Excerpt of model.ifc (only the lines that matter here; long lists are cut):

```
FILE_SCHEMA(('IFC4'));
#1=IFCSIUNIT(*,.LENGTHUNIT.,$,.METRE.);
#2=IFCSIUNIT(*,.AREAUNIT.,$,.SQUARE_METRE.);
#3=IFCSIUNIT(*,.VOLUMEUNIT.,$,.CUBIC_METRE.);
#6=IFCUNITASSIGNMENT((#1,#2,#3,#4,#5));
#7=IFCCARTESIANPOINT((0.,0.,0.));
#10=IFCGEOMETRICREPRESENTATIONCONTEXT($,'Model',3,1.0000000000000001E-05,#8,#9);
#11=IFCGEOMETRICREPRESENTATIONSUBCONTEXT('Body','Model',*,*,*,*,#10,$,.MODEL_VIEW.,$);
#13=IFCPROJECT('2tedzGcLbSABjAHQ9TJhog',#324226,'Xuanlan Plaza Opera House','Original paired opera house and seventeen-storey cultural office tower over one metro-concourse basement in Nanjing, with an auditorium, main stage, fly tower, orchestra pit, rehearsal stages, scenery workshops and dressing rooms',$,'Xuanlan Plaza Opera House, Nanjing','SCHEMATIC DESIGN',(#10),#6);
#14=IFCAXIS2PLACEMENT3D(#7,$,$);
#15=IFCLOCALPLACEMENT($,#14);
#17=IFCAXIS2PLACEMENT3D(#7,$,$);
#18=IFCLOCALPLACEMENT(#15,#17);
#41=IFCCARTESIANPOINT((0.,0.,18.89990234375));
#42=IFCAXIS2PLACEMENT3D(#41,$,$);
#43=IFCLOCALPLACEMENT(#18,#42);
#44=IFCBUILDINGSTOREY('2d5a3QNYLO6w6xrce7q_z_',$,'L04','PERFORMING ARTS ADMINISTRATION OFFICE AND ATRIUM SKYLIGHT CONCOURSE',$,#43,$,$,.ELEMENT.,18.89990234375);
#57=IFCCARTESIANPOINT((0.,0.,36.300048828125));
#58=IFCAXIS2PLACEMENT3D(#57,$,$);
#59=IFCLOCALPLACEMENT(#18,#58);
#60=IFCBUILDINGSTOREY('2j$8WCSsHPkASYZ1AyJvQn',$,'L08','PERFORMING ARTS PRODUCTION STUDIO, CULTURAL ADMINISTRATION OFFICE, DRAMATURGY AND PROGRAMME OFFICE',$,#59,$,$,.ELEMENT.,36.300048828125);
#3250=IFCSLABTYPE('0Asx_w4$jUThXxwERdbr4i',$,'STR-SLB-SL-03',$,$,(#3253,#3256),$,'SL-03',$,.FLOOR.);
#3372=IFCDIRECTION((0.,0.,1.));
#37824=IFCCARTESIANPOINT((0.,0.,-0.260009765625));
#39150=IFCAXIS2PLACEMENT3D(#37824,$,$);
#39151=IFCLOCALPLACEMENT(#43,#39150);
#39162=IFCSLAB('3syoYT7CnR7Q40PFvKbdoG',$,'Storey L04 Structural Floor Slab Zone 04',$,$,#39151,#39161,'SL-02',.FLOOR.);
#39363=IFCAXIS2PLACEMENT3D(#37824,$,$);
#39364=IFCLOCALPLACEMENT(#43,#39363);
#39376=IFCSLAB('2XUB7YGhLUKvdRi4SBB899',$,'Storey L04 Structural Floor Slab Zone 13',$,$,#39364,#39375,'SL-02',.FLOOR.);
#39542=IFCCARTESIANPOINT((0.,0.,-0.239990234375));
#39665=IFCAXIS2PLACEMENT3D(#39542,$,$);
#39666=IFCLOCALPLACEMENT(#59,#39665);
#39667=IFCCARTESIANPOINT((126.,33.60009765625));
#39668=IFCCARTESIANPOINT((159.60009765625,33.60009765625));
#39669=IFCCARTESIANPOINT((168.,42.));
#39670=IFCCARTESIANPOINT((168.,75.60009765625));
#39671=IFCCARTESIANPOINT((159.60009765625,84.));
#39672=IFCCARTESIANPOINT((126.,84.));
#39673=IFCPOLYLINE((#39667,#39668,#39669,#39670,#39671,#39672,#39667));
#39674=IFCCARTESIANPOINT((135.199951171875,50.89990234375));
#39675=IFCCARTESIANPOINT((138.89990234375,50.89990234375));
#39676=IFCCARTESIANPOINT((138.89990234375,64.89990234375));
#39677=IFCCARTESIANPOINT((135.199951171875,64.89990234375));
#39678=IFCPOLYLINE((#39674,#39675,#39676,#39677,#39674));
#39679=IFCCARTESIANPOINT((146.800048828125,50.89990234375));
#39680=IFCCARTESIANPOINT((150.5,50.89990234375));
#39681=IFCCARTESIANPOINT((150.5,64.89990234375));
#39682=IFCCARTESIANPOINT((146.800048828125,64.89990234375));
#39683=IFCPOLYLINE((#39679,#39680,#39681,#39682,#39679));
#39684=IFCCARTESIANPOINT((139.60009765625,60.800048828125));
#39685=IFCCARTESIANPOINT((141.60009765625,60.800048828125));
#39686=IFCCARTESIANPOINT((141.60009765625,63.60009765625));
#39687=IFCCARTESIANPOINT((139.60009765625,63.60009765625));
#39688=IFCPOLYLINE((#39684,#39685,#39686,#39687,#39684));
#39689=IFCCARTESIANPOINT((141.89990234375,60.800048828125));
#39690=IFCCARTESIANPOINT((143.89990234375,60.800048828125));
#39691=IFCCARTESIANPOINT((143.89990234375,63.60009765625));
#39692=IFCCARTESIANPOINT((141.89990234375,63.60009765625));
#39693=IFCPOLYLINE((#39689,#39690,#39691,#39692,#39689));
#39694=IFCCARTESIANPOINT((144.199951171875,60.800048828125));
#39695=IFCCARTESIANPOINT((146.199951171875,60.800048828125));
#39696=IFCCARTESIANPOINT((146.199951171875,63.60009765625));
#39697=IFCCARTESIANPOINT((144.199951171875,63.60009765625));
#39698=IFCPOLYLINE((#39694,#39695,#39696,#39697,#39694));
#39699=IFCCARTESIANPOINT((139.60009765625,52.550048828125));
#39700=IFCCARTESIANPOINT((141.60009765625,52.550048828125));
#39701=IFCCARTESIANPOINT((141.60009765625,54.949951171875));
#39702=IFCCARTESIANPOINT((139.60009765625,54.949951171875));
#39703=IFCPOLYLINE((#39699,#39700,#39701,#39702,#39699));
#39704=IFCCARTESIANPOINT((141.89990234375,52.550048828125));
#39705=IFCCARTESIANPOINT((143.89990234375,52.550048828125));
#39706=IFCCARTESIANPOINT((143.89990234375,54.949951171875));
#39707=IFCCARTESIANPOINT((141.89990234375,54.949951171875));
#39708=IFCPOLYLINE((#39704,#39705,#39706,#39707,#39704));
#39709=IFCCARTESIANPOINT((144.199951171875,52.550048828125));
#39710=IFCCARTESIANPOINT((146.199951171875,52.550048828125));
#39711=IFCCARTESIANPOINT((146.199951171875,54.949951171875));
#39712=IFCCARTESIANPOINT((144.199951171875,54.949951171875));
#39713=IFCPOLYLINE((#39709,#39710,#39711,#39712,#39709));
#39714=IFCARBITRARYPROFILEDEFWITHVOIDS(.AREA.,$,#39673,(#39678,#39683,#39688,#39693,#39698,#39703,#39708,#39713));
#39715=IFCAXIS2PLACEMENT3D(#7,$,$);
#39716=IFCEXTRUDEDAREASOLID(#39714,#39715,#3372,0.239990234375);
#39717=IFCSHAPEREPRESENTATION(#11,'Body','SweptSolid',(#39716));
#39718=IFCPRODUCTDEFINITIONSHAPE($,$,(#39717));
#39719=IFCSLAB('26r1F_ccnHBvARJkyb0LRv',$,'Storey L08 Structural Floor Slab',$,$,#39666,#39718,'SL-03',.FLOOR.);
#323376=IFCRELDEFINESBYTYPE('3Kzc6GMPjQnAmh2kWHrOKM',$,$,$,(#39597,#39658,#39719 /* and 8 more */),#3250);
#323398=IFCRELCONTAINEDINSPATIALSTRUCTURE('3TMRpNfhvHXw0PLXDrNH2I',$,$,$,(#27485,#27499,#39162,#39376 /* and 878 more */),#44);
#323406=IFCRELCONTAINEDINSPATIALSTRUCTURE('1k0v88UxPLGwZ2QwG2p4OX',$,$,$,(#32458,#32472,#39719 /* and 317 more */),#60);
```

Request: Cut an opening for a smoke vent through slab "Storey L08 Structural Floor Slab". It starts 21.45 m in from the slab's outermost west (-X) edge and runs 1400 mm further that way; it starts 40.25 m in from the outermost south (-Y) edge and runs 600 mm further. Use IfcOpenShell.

```python
import numpy as np
import ifcopenshell
import ifcopenshell.api.feature
import ifcopenshell.api.geometry
import ifcopenshell.api.root
import ifcopenshell.geom
import ifcopenshell.util.placement
import ifcopenshell.util.representation
import ifcopenshell.util.shape
import ifcopenshell.util.unit

model = ifcopenshell.open("model.ifc")
unit_scale = ifcopenshell.util.unit.calculate_unit_scale(model)
settings = ifcopenshell.geom.settings()


def volume(element):
    """Net volume in cubic metres, openings subtracted."""
    shape = ifcopenshell.geom.create_shape(settings, element)
    return ifcopenshell.util.shape.get_volume(shape.geometry)


slab = model.by_id(39719)
before = volume(slab)

# Extent in the slab's own axes, in metres. The edges named are its -X and -Y sides.
slab_shape = ifcopenshell.geom.create_shape(settings, slab)
vertices = ifcopenshell.util.shape.get_vertices(slab_shape.geometry)
x_min, y_min, bottom = vertices.min(axis=0)
top = vertices[:, 2].max()

opening = ifcopenshell.api.root.create_entity(model, ifc_class="IfcOpeningElement", name="Smoke vent opening", predefined_type="OPENING")
context = ifcopenshell.util.representation.get_context(model, "Model", "Body", "MODEL_VIEW")
width, depth = 1.4, 0.6
outline = [(0.0, 0.0), (width, 0.0), (width, depth), (0.0, depth), (0.0, 0.0)]
# Overshoot both faces by 50 mm so the cut is clean.
shape = ifcopenshell.api.geometry.add_slab_representation(
    model, context=context, depth=top - bottom + 0.1, polyline=outline
)
ifcopenshell.api.geometry.assign_representation(model, product=opening, representation=shape)

matrix = ifcopenshell.util.placement.get_local_placement(slab.ObjectPlacement)
matrix[:, 3] = matrix @ np.append(np.array([x_min + 21.45, y_min + 40.25, bottom - 0.05]) / unit_scale, 1.0)
ifcopenshell.api.geometry.edit_object_placement(model, product=opening, matrix=matrix, is_si=False)
ifcopenshell.api.feature.add_feature(model, feature=opening, element=slab)

after = volume(slab)

print(f"slab volume {before:.3f} -> {after:.3f} m3")

model.write("model_updated.ifc")
```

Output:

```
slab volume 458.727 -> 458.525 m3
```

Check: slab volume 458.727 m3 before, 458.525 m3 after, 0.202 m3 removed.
